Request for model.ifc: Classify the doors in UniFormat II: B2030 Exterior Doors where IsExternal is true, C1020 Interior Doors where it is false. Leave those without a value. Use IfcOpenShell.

First a look at what the model holds.

```python
import ifcopenshell
import ifcopenshell.util.element

model = ifcopenshell.open("model.ifc")
print(model.schema)
print("classifications:", [c.Name for c in model.by_type("IfcClassification")])
values = [ifcopenshell.util.element.get_pset(e, "Pset_DoorCommon", "IsExternal") for e in model.by_type("IfcDoor")]
for value in (True, False, None):
    print("IsExternal", value, values.count(value))
```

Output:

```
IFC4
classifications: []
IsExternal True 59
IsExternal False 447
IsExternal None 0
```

```python
import ifcopenshell
import ifcopenshell.api.classification
import ifcopenshell.util.element

model = ifcopenshell.open("model.ifc")

system = ifcopenshell.api.classification.add_classification(model, classification="UniFormat II")

doors = model.by_type("IfcDoor")
external = {e: ifcopenshell.util.element.get_pset(e, "Pset_DoorCommon", "IsExternal") for e in doors}
for flag, code, name in ((True, "B2030", "Exterior Doors"), (False, "C1020", "Interior Doors")):
    products = [e for e in doors if external[e] is flag]
    ifcopenshell.api.classification.add_reference(
        model, products=products, classification=system, identification=code, name=name
    )
    print(code, len(products))

model.write("model_rev.ifc")
```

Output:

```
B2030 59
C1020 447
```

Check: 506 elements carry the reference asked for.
